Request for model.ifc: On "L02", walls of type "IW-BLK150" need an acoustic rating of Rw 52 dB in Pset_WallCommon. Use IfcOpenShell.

First a look at what the model holds.

```python
import ifcopenshell
import ifcopenshell.util.element

model = ifcopenshell.open("model.ifc")
print(model.schema)
storey = next(s for s in model.by_type("IfcBuildingStorey") if s.Name == "L02")
walls = [e for e in ifcopenshell.util.element.get_decomposition(storey) if e.is_a("IfcWall")]
seen = {}
for e in walls:
    element_type = ifcopenshell.util.element.get_type(e)
    key = (element_type.Name if element_type != e and element_type else None, ifcopenshell.util.element.get_pset(e, "Pset_WallCommon", "AcousticRating"))
    seen[key] = seen.get(key, 0) + 1
for (name, value), count in sorted(seen.items(), key=str):
    print(count, "x", name, "|", value)
```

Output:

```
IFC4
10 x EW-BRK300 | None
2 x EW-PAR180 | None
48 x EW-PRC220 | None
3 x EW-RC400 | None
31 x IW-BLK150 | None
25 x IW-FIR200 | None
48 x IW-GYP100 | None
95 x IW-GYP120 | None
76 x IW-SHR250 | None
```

```python
import ifcopenshell
import ifcopenshell.api.pset
import ifcopenshell.util.element

model = ifcopenshell.open("model.ifc")

storey = next(s for s in model.by_type("IfcBuildingStorey") if s.Name == "L02")
walls = [e for e in ifcopenshell.util.element.get_decomposition(storey) if e.is_a("IfcWall")]

count = 0
for e in walls:
    element_type = ifcopenshell.util.element.get_type(e)
    if element_type in (None, e) or element_type.Name != "IW-BLK150":
        continue
    # add_pset returns the element's existing set when there is one.
    pset = ifcopenshell.api.pset.add_pset(model, product=e, name="Pset_WallCommon")
    ifcopenshell.api.pset.edit_pset(model, pset=pset, properties={"AcousticRating": "Rw 52 dB"})
    count += 1

print(count, "walls updated")

model.write("model_rev.ifc")
```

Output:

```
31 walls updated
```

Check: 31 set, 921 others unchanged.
